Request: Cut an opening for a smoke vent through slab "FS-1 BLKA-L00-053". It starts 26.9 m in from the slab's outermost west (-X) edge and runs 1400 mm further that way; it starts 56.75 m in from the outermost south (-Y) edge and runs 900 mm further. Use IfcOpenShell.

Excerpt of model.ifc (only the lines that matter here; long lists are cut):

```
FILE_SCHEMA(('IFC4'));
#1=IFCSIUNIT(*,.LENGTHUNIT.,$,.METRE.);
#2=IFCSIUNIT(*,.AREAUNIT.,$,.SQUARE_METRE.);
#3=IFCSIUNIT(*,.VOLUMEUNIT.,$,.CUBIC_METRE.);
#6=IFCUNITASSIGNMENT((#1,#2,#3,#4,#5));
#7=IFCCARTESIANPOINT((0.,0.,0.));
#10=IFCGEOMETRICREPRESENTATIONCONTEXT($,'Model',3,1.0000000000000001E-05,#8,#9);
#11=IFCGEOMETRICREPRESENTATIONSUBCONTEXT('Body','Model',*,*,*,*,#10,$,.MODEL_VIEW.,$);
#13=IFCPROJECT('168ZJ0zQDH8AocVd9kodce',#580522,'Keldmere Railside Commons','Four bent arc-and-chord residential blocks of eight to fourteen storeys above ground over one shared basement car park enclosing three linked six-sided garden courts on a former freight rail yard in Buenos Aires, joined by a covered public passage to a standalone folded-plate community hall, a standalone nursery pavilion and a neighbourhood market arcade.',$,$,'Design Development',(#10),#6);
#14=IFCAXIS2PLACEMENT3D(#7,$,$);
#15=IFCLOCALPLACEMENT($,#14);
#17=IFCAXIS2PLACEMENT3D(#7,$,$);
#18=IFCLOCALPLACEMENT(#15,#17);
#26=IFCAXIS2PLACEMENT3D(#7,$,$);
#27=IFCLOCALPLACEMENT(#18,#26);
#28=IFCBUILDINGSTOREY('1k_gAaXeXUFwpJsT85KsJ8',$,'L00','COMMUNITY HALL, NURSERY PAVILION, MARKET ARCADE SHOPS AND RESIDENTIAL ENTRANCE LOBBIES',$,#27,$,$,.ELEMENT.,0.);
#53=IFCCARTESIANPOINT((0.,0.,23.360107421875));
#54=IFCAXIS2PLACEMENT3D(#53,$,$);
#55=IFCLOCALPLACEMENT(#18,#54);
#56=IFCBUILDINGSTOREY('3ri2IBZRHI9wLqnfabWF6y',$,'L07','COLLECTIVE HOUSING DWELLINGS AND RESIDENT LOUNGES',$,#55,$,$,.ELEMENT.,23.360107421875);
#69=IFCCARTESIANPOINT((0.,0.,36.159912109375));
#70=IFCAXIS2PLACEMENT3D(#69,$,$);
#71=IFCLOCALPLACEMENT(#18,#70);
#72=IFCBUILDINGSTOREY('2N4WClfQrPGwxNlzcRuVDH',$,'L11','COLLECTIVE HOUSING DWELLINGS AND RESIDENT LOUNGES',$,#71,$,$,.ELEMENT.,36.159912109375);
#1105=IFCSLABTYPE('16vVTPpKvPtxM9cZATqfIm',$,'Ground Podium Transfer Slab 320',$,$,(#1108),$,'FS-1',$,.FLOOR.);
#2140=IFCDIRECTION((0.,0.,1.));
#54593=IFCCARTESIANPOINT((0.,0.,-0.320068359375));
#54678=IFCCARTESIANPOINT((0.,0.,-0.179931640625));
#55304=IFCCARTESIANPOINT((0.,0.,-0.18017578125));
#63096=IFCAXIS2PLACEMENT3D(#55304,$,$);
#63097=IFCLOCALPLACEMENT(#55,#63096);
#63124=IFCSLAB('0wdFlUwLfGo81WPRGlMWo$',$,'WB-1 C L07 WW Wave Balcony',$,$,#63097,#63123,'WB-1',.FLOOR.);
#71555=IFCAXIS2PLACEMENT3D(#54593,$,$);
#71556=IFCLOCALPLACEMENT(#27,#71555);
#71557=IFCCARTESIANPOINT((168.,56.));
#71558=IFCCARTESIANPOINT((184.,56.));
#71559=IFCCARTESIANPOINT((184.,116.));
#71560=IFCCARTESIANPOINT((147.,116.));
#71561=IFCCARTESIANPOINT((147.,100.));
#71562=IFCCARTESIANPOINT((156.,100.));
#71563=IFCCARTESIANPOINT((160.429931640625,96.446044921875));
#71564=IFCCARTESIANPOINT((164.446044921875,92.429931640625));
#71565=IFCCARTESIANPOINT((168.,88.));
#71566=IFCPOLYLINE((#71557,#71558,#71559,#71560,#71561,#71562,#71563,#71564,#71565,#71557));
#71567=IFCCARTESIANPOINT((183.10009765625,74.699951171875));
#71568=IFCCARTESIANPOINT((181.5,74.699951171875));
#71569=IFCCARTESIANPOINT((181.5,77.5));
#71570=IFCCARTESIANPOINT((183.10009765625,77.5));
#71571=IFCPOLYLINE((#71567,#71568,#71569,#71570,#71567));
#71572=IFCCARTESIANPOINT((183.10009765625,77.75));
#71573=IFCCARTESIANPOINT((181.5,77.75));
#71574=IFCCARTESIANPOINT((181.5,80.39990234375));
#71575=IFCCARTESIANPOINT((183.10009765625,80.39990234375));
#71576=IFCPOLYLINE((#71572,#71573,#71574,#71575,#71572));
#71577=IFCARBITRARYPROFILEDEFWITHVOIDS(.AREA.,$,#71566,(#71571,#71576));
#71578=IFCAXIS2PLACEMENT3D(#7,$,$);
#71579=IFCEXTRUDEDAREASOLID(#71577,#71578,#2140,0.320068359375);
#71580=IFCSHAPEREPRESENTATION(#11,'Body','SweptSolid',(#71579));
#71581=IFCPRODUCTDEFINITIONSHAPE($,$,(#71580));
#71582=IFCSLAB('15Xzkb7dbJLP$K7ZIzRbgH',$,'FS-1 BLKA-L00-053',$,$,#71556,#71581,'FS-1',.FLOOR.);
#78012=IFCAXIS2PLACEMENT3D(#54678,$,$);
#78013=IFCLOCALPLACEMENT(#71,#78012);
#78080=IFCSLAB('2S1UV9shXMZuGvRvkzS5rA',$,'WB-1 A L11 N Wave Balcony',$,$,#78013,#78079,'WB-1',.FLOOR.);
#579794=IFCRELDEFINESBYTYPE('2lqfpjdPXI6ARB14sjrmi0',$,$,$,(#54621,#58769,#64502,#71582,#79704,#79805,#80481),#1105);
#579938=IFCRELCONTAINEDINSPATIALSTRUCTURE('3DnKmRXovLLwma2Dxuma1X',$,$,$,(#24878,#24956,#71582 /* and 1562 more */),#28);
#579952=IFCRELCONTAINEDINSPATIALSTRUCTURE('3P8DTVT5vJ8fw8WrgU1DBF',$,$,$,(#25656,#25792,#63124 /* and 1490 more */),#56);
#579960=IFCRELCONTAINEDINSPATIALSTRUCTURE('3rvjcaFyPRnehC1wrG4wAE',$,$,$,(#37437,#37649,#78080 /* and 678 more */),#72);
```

```python
import numpy as np
import ifcopenshell
import ifcopenshell.api.feature
import ifcopenshell.api.geometry
import ifcopenshell.api.root
import ifcopenshell.geom
import ifcopenshell.util.placement
import ifcopenshell.util.representation
import ifcopenshell.util.shape
import ifcopenshell.util.unit

model = ifcopenshell.open("model.ifc")
unit_scale = ifcopenshell.util.unit.calculate_unit_scale(model)
settings = ifcopenshell.geom.settings()


def volume(element):
    """Net volume in cubic metres, openings subtracted."""
    shape = ifcopenshell.geom.create_shape(settings, element)
    return ifcopenshell.util.shape.get_volume(shape.geometry)


slab = model.by_guid("15Xzkb7dbJLP$K7ZIzRbgH")
before = volume(slab)

# Extent in the slab's own axes, in metres. The edges named are its -X and -Y sides.
slab_shape = ifcopenshell.geom.create_shape(settings, slab)
vertices = ifcopenshell.util.shape.get_vertices(slab_shape.geometry)
x_min, y_min, bottom = vertices.min(axis=0)
top = vertices[:, 2].max()

opening = ifcopenshell.api.root.create_entity(model, ifc_class="IfcOpeningElement", name="Smoke vent opening", predefined_type="OPENING")
context = ifcopenshell.util.representation.get_context(model, "Model", "Body", "MODEL_VIEW")
width, depth = 1.4, 0.9
outline = [(0.0, 0.0), (width, 0.0), (width, depth), (0.0, depth), (0.0, 0.0)]
# Overshoot both faces by 50 mm so the cut is clean.
shape = ifcopenshell.api.geometry.add_slab_representation(
    model, context=context, depth=top - bottom + 0.1, polyline=outline
)
ifcopenshell.api.geometry.assign_representation(model, product=opening, representation=shape)

matrix = ifcopenshell.util.placement.get_local_placement(slab.ObjectPlacement)
matrix[:, 3] = matrix @ np.append(np.array([x_min + 26.9, y_min + 56.75, bottom - 0.05]) / unit_scale, 1.0)
ifcopenshell.api.geometry.edit_object_placement(model, product=opening, matrix=matrix, is_si=False)
ifcopenshell.api.feature.add_feature(model, feature=opening, element=slab)

after = volume(slab)

print(f"slab volume {before:.3f} -> {after:.3f} m3")

model.write("model_v2.ifc")
```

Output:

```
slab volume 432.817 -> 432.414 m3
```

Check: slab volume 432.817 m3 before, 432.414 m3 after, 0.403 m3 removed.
